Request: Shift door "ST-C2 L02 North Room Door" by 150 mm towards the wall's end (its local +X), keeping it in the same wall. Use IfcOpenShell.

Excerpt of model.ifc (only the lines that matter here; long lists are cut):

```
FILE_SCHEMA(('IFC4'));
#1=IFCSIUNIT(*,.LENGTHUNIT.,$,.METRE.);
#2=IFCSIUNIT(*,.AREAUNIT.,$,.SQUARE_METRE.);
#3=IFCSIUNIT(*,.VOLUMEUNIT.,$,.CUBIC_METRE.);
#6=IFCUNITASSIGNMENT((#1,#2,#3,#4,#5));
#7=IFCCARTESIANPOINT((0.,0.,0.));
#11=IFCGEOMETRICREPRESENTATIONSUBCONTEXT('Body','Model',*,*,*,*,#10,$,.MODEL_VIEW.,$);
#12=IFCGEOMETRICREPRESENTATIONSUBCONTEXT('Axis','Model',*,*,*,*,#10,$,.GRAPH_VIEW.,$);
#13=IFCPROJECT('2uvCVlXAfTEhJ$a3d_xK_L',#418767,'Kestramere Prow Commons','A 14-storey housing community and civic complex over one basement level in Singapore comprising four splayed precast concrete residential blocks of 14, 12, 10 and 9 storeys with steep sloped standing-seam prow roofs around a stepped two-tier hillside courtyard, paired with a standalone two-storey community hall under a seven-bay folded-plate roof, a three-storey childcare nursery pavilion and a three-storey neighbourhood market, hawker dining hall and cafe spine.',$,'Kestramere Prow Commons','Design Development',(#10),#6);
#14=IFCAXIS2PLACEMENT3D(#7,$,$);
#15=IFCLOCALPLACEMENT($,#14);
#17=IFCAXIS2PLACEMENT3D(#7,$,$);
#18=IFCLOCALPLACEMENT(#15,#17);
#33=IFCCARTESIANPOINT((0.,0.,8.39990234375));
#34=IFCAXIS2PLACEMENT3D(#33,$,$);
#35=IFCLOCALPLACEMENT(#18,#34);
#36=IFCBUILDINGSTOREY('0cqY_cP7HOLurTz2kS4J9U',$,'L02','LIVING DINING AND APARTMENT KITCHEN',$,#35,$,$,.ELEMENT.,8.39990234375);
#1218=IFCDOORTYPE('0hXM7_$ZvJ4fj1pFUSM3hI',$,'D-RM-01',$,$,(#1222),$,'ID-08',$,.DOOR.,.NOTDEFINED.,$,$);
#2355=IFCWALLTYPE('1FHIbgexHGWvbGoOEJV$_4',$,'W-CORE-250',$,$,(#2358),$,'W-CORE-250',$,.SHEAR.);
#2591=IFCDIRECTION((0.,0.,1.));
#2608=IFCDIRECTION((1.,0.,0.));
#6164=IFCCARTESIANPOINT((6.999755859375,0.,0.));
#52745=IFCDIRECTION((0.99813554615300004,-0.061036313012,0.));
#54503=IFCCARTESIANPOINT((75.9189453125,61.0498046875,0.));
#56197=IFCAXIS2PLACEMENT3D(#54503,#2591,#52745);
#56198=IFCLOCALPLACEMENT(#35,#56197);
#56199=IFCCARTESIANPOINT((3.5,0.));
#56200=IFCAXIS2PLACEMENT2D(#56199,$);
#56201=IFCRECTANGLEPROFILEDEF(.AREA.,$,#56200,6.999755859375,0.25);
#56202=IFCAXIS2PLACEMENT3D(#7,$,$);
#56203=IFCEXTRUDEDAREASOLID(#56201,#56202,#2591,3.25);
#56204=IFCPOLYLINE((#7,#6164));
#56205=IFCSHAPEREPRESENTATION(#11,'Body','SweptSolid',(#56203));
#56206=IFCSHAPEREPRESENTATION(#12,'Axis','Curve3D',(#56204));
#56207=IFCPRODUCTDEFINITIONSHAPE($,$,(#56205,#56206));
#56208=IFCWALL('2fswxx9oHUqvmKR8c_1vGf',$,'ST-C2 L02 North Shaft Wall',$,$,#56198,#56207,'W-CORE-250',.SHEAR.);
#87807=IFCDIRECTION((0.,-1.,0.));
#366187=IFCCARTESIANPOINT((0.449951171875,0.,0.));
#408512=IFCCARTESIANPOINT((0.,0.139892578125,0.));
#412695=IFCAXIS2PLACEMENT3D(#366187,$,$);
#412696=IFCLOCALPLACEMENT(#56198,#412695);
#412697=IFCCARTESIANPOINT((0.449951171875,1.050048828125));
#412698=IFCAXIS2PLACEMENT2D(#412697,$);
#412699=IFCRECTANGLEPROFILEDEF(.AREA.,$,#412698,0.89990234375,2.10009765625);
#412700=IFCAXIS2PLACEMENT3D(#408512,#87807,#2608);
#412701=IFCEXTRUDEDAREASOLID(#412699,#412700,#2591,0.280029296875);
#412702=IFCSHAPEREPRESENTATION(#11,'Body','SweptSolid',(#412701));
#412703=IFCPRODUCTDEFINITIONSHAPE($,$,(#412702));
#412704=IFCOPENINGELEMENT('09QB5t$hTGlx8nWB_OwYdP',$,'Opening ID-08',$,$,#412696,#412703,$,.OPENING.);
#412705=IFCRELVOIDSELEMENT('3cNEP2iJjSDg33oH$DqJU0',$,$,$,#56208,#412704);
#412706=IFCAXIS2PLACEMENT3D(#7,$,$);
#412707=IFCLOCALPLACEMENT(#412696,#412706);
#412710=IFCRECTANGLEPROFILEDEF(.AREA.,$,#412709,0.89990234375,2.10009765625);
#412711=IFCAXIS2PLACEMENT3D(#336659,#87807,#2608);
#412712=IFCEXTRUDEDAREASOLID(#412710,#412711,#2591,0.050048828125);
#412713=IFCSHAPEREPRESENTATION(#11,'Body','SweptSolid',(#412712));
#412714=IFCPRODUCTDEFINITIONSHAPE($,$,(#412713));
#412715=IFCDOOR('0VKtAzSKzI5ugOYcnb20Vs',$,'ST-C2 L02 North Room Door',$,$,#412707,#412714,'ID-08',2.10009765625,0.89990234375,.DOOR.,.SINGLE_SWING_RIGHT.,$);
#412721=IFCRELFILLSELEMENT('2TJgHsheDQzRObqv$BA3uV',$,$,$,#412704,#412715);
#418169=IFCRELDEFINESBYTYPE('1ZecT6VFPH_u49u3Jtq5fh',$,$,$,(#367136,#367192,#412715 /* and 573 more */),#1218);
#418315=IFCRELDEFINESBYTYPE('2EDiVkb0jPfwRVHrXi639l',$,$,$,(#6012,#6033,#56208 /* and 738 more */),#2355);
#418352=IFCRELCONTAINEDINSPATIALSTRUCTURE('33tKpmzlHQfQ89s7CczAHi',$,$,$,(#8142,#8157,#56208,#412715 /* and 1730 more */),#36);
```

```python
import ifcopenshell
import ifcopenshell.api.geometry
import ifcopenshell.util.placement
import ifcopenshell.util.unit

model = ifcopenshell.open("model.ifc")
unit_scale = ifcopenshell.util.unit.calculate_unit_scale(model)

door = model.by_id(412715)
opening = door.FillsVoids[0].RelatingOpeningElement
wall = opening.VoidsElements[0].RelatingBuildingElement

wall_matrix = ifcopenshell.util.placement.get_local_placement(wall.ObjectPlacement)
shift = wall_matrix[:3, 0] * 0.15 / unit_scale
before = ifcopenshell.util.placement.get_local_placement(door.ObjectPlacement)[:3, 3].copy()

# The door is placed relative to its opening, so it follows when the opening moves.
matrix = ifcopenshell.util.placement.get_local_placement(opening.ObjectPlacement)
matrix[:3, 3] += shift
ifcopenshell.api.geometry.edit_object_placement(
    model, product=opening, matrix=matrix, is_si=False, should_transform_children=True
)

after = ifcopenshell.util.placement.get_local_placement(door.ObjectPlacement)[:3, 3]
print("door moved by", (after - before).round(3) + 0.0)

model.write("model_rev.ifc")
```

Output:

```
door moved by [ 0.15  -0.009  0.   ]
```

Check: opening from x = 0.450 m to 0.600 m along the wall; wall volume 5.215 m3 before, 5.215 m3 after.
